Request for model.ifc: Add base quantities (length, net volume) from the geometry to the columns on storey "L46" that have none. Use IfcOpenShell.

First a look at what the model holds.

```python
import ifcopenshell
import ifcopenshell.util.element
import ifcopenshell.util.unit

model = ifcopenshell.open("model.ifc")
print(model.schema)
for unit_type in ("LENGTHUNIT", "AREAUNIT", "VOLUMEUNIT"):
    print(unit_type, ifcopenshell.util.unit.calculate_unit_scale(model, unit_type))
storey = next(s for s in model.by_type("IfcBuildingStorey") if s.Name == "L46")
columns = [e for e in ifcopenshell.util.element.get_decomposition(storey) if e.is_a("IfcColumn")]
for e in sorted(columns, key=lambda e: e.id()):
    print(e.id(), e.is_a(), e.Name, list(ifcopenshell.util.element.get_psets(e, qtos_only=True)), sep=" | ")
```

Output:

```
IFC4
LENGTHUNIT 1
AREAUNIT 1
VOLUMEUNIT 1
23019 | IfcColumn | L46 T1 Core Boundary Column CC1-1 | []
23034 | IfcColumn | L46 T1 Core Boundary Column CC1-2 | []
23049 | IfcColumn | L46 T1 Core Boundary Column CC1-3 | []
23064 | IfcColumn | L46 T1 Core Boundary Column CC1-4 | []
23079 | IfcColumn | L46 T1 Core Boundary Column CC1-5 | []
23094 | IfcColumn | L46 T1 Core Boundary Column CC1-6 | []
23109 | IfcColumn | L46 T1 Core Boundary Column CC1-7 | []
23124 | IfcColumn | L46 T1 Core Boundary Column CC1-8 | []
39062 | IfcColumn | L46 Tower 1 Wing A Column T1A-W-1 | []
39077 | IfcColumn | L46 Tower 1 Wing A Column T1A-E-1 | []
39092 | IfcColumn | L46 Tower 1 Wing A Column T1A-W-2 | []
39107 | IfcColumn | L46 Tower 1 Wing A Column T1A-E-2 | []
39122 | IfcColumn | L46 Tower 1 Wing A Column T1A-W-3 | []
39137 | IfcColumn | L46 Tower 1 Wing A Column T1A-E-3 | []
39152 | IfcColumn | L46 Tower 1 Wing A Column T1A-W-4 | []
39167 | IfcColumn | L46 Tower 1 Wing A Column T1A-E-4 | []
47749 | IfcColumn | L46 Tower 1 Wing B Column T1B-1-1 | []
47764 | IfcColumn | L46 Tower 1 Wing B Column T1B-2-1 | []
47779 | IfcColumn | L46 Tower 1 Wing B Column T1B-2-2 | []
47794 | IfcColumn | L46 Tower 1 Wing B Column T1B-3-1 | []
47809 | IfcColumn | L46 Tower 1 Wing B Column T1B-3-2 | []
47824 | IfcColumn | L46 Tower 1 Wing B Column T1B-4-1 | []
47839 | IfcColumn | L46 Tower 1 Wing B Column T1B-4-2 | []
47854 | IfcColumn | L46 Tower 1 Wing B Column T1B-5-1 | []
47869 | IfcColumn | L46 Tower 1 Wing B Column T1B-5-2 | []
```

```python
import ifcopenshell
import ifcopenshell.api.pset
import ifcopenshell.geom
import ifcopenshell.util.element
import ifcopenshell.util.shape
import ifcopenshell.util.unit

model = ifcopenshell.open("model.ifc")
unit_scale = ifcopenshell.util.unit.calculate_unit_scale(model)
volume_scale = ifcopenshell.util.unit.calculate_unit_scale(model, "VOLUMEUNIT")
settings = ifcopenshell.geom.settings()

storey = next(s for s in model.by_type("IfcBuildingStorey") if s.Name == "L46")
columns = [e for e in ifcopenshell.util.element.get_decomposition(storey) if e.is_a("IfcColumn")]

for e in sorted(columns, key=lambda e: e.id()):
    if ifcopenshell.util.element.get_psets(e, qtos_only=True, should_inherit=False):
        continue
    # Geometry comes back in metres, in the element's own axes.
    shape = ifcopenshell.geom.create_shape(settings, e)
    values = {
        "Length": ifcopenshell.util.shape.get_z(shape.geometry) / unit_scale,
        "NetVolume": ifcopenshell.util.shape.get_volume(shape.geometry) / volume_scale,
    }
    qto = ifcopenshell.api.pset.add_qto(model, product=e, name="Qto_ColumnBaseQuantities")
    ifcopenshell.api.pset.edit_qto(model, qto=qto, properties=values)
    print(e.id(), {k: round(v, 3) for k, v in values.items()})

model.write("model_v2.ifc")
```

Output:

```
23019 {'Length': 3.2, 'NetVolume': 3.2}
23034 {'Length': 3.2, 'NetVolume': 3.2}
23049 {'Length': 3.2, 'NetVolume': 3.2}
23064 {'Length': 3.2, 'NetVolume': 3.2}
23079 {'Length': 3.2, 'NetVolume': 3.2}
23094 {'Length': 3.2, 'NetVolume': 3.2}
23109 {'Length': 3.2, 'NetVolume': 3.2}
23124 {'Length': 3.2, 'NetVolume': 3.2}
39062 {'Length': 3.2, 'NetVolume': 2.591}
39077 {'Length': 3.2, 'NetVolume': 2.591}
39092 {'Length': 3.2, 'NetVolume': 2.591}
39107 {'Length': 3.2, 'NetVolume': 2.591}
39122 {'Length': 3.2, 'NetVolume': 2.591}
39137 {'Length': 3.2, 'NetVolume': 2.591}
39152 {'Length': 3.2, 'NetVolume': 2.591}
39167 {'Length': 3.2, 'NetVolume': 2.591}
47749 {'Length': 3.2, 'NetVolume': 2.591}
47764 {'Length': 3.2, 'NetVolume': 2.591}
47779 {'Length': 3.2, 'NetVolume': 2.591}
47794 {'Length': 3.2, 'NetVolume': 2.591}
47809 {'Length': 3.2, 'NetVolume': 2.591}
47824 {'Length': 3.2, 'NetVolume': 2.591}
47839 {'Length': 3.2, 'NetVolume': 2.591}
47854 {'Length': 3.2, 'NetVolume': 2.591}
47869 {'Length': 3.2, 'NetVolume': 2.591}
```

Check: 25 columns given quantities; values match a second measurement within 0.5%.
